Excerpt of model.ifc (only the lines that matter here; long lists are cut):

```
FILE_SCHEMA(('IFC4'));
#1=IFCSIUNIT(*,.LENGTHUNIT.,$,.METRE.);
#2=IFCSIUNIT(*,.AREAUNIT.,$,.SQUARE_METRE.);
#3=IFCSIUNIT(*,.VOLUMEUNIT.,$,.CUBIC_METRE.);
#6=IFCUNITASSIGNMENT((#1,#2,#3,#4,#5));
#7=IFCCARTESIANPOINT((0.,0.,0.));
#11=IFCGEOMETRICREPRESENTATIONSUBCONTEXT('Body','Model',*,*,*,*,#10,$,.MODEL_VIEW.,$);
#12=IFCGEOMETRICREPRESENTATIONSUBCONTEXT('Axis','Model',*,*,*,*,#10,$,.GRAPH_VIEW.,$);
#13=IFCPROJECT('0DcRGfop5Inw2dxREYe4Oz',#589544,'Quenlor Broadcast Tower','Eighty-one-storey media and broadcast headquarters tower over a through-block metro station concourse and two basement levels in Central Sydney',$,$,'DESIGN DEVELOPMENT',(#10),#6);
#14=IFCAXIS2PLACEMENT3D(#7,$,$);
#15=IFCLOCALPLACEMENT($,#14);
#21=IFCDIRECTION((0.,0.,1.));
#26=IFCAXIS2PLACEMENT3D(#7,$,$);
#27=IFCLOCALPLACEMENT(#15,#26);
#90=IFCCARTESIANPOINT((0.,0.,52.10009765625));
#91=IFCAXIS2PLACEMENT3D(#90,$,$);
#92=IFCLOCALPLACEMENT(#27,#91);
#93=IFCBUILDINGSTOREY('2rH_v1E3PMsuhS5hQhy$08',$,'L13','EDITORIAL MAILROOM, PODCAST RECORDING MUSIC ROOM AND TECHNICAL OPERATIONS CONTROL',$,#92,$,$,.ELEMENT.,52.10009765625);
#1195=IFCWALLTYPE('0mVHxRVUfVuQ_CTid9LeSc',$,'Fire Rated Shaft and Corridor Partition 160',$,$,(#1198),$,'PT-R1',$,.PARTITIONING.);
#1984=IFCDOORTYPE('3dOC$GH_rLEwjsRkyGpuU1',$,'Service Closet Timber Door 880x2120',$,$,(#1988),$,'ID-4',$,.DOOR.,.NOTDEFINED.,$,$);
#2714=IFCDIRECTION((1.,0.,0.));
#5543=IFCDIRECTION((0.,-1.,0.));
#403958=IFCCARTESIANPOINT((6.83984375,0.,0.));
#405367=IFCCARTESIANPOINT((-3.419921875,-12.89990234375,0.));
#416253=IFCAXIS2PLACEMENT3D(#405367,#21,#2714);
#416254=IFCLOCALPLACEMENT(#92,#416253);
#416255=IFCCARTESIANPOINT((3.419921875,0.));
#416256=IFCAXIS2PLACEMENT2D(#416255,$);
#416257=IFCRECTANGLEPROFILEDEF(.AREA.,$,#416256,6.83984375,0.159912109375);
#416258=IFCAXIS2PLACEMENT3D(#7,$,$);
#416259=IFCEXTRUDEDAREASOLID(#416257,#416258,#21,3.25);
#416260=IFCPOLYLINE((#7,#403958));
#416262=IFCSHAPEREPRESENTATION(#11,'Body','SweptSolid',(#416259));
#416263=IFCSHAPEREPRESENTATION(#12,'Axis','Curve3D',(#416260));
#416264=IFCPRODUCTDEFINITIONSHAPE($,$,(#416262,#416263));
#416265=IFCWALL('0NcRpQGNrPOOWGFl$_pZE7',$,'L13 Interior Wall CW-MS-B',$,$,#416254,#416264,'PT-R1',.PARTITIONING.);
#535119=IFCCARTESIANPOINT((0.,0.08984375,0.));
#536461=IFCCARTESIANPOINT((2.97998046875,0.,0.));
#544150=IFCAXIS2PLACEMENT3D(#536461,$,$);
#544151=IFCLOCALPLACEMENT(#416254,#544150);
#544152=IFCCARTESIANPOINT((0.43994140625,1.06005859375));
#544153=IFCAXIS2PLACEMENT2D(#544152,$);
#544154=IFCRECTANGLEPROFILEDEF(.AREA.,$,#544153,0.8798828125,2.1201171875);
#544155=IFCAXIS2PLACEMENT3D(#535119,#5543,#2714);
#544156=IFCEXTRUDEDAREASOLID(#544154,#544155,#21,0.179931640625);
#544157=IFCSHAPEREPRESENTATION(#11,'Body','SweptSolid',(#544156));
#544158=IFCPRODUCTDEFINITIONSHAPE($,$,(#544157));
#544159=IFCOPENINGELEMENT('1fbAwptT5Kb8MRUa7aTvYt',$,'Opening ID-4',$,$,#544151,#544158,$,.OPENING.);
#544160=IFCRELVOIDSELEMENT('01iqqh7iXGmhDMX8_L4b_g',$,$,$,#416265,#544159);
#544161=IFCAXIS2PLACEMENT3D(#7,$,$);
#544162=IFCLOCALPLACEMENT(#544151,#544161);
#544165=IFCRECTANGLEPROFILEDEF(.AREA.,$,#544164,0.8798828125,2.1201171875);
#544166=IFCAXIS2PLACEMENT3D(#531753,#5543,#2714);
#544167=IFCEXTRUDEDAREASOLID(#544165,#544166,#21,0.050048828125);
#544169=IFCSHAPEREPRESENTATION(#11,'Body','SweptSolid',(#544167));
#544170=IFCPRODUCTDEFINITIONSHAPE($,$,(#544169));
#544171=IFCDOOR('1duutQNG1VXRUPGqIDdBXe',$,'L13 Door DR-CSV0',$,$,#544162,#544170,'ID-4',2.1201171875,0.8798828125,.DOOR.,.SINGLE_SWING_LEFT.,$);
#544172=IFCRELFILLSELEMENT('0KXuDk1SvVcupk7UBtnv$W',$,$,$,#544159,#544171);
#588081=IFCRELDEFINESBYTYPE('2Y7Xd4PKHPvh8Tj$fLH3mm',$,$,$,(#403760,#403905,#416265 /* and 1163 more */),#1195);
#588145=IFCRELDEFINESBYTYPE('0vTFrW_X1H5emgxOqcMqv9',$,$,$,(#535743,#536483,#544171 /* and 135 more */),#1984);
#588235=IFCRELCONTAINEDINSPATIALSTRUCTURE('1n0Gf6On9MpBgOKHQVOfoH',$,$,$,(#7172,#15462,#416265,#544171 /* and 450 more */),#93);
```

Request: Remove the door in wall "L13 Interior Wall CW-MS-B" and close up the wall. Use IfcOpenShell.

```python
import ifcopenshell
import ifcopenshell.api.feature
import ifcopenshell.api.root
import ifcopenshell.geom
import ifcopenshell.util.shape

model = ifcopenshell.open("model.ifc")
settings = ifcopenshell.geom.settings()


def volume(element):
    """Net volume in cubic metres, openings subtracted."""
    shape = ifcopenshell.geom.create_shape(settings, element)
    return ifcopenshell.util.shape.get_volume(shape.geometry)


door = model.by_guid("1duutQNG1VXRUPGqIDdBXe")
opening = door.FillsVoids[0].RelatingOpeningElement
wall = opening.VoidsElements[0].RelatingBuildingElement
before = volume(wall)

ifcopenshell.api.root.remove_product(model, product=door)
ifcopenshell.api.feature.remove_feature(model, feature=opening)

after = volume(wall)

print(f"wall volume {before:.3f} -> {after:.3f} m3")

model.write("model_v2.ifc")
```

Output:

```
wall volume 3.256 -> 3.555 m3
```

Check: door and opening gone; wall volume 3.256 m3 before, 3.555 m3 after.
